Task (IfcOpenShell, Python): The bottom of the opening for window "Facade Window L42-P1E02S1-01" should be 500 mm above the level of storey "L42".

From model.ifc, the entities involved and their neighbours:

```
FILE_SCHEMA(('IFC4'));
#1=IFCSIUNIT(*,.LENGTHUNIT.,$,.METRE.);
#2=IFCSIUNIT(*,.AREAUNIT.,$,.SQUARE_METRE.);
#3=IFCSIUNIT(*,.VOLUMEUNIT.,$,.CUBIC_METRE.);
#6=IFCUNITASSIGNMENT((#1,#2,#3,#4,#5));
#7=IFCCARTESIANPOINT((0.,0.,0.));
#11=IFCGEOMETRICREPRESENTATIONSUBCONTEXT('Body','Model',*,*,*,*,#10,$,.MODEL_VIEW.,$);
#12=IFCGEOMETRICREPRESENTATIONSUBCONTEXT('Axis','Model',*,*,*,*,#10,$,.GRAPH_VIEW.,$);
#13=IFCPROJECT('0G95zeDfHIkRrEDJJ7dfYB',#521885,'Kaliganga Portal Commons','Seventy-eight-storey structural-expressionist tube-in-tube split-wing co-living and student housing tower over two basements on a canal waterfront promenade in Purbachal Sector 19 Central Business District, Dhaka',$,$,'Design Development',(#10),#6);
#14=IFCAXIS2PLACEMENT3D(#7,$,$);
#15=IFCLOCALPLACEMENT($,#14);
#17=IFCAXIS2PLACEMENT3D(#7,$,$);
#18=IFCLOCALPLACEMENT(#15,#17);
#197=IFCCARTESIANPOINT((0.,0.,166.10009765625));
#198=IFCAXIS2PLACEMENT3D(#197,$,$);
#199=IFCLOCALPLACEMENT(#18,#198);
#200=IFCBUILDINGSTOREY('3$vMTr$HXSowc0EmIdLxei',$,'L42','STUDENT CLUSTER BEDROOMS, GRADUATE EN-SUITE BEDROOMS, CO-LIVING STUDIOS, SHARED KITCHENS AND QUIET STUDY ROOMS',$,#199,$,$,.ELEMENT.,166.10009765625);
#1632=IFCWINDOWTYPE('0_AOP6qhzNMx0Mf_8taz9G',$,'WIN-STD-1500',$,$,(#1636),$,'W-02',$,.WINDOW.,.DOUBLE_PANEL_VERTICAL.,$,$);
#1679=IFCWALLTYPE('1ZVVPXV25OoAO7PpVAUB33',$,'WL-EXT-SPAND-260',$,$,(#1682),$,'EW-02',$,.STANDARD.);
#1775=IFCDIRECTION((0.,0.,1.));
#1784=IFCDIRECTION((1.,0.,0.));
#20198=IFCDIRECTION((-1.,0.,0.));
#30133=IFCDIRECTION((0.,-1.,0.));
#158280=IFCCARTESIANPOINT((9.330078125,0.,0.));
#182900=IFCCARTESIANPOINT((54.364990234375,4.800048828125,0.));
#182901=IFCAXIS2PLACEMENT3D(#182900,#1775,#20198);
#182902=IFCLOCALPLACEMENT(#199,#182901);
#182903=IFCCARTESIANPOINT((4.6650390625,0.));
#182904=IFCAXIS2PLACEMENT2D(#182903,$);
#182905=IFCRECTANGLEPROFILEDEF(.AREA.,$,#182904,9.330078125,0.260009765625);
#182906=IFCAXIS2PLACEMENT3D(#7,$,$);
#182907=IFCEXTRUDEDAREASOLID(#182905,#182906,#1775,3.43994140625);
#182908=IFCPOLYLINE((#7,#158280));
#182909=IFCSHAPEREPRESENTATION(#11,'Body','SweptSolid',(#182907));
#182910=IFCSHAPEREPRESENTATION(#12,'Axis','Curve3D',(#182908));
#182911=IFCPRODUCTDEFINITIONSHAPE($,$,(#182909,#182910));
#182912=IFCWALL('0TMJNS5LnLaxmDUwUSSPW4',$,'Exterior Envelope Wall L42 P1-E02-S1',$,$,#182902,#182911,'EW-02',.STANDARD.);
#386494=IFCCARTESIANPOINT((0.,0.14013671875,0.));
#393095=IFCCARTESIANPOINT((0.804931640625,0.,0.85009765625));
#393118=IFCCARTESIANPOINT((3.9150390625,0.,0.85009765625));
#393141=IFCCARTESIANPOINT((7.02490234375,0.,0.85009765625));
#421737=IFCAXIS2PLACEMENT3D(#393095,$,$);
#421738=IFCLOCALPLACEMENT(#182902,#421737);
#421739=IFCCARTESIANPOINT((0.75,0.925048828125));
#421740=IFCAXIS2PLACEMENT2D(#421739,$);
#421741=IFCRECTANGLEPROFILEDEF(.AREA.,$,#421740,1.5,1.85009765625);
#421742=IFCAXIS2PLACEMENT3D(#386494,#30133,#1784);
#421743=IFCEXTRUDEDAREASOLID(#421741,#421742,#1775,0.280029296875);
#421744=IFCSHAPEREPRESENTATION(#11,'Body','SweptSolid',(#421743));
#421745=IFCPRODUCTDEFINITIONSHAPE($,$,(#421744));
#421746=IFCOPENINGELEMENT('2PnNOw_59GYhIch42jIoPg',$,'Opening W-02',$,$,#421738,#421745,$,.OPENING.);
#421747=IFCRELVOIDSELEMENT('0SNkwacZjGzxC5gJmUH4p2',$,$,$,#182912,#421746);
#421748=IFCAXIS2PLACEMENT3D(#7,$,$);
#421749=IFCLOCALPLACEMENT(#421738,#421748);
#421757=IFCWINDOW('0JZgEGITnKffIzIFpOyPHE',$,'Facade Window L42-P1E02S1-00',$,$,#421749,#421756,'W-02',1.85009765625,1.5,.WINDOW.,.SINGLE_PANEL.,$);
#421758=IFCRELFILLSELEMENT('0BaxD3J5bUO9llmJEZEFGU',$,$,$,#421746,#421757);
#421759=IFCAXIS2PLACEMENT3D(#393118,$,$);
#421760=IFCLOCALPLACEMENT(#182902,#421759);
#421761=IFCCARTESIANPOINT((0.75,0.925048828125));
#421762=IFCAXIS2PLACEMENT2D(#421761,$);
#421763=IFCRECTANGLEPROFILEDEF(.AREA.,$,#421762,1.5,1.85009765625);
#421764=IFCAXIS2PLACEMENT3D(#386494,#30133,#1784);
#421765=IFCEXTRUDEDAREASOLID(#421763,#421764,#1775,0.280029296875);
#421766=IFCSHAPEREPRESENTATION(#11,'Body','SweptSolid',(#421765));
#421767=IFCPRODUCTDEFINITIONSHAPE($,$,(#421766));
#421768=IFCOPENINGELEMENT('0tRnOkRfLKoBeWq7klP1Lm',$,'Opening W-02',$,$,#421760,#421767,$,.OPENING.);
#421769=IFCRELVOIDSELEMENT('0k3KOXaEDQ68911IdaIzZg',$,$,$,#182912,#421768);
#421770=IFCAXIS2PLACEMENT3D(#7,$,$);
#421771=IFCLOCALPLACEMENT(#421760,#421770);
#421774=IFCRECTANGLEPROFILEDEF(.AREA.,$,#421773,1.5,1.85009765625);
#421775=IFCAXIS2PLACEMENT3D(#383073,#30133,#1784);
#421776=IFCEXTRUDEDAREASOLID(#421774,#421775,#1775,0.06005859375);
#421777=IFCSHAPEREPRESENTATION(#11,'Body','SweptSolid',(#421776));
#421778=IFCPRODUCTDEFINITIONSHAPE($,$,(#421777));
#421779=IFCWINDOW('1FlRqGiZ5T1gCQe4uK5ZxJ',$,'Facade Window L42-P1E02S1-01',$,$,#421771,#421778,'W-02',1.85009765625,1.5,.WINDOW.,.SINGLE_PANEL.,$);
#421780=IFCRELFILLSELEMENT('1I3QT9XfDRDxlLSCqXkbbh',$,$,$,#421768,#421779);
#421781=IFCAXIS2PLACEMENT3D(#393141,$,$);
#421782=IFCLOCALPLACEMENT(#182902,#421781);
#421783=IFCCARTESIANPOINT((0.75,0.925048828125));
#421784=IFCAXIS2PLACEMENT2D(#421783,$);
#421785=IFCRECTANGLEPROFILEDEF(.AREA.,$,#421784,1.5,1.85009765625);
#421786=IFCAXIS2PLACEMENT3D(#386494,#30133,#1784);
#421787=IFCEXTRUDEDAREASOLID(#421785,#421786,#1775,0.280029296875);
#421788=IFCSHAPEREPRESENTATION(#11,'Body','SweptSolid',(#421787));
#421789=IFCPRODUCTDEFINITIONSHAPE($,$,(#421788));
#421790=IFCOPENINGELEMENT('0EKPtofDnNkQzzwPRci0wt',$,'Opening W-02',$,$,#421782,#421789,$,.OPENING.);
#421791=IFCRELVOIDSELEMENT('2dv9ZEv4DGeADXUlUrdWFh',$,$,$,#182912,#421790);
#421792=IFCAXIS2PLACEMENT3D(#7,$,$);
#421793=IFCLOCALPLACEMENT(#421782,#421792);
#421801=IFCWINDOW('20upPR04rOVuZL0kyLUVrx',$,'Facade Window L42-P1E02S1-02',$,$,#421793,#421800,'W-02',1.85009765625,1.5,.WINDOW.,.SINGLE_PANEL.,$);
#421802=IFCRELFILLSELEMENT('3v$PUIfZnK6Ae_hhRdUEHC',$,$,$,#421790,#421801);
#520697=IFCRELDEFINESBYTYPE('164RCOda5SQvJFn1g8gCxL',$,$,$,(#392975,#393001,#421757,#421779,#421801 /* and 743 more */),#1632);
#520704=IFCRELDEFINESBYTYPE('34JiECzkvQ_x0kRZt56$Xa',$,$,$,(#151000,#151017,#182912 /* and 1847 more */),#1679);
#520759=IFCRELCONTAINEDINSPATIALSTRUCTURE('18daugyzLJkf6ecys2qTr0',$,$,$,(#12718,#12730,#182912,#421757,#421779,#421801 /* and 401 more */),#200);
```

```python
import numpy as np
import ifcopenshell
import ifcopenshell.api.geometry
import ifcopenshell.geom
import ifcopenshell.util.element
import ifcopenshell.util.placement
import ifcopenshell.util.shape
import ifcopenshell.util.unit

model = ifcopenshell.open("model.ifc")
unit_scale = ifcopenshell.util.unit.calculate_unit_scale(model)

window = model.by_id(421779)
opening = window.FillsVoids[0].RelatingOpeningElement
storey = ifcopenshell.util.element.get_container(window, ifc_class="IfcBuildingStorey")
level = ifcopenshell.util.placement.get_local_placement(storey.ObjectPlacement)[2, 3]

# The opening's origin need not be at the sill, so measure its lowest point.
shape = ifcopenshell.geom.create_shape(ifcopenshell.geom.settings(), opening)
bottom = ifcopenshell.util.shape.get_shape_bottom_elevation(shape, shape.geometry) / unit_scale
dz = level + 0.5 / unit_scale - bottom

shift = np.array([0.0, 0.0, dz])
# The window is placed relative to its opening, so it follows when the opening moves.
matrix = ifcopenshell.util.placement.get_local_placement(opening.ObjectPlacement)
matrix[:3, 3] += shift
ifcopenshell.api.geometry.edit_object_placement(
    model, product=opening, matrix=matrix, is_si=False, should_transform_children=True
)

print(f"moved by {dz * unit_scale:+.3f} m")

model.write("model_rev.ifc")
```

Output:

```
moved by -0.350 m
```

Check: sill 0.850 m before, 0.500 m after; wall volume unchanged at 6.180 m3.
